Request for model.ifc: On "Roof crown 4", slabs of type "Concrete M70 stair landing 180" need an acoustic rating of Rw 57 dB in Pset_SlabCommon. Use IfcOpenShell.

First a look at what the model holds.

```python
import ifcopenshell
import ifcopenshell.util.element

model = ifcopenshell.open("model.ifc")
print(model.schema)
storey = next(s for s in model.by_type("IfcBuildingStorey") if s.Name == "Roof crown 4")
slabs = [e for e in ifcopenshell.util.element.get_decomposition(storey) if e.is_a("IfcSlab")]
seen = {}
for e in slabs:
    element_type = ifcopenshell.util.element.get_type(e)
    key = (element_type.Name if element_type != e and element_type else None, ifcopenshell.util.element.get_pset(e, "Pset_SlabCommon", "AcousticRating"))
    seen[key] = seen.get(key, 0) + 1
for (name, value), count in sorted(seen.items(), key=str):
    print(count, "x", name, "|", value)
```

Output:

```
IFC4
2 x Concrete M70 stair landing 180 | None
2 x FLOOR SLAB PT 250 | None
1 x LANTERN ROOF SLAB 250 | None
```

```python
import ifcopenshell
import ifcopenshell.api.pset
import ifcopenshell.util.element

model = ifcopenshell.open("model.ifc")

storey = next(s for s in model.by_type("IfcBuildingStorey") if s.Name == "Roof crown 4")
slabs = [e for e in ifcopenshell.util.element.get_decomposition(storey) if e.is_a("IfcSlab")]

count = 0
for e in slabs:
    element_type = ifcopenshell.util.element.get_type(e)
    if element_type in (None, e) or element_type.Name != "Concrete M70 stair landing 180":
        continue
    # add_pset returns the element's existing set when there is one.
    pset = ifcopenshell.api.pset.add_pset(model, product=e, name="Pset_SlabCommon")
    ifcopenshell.api.pset.edit_pset(model, pset=pset, properties={"AcousticRating": "Rw 57 dB"})
    count += 1

print(count, "slabs updated")

model.write("model_rev.ifc")
```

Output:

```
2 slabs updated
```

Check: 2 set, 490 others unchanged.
